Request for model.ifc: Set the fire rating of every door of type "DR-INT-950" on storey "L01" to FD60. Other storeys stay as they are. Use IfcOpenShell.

First a look at what the model holds.

```python
import ifcopenshell
import ifcopenshell.util.element

model = ifcopenshell.open("model.ifc")
print(model.schema)
storey = next(s for s in model.by_type("IfcBuildingStorey") if s.Name == "L01")
doors = [e for e in ifcopenshell.util.element.get_decomposition(storey) if e.is_a("IfcDoor")]
seen = {}
for e in doors:
    element_type = ifcopenshell.util.element.get_type(e)
    key = (element_type.Name if element_type != e and element_type else None, ifcopenshell.util.element.get_pset(e, "Pset_DoorCommon", "FireRating"))
    seen[key] = seen.get(key, 0) + 1
for (name, value), count in sorted(seen.items(), key=str):
    print(count, "x", name, "|", value)
```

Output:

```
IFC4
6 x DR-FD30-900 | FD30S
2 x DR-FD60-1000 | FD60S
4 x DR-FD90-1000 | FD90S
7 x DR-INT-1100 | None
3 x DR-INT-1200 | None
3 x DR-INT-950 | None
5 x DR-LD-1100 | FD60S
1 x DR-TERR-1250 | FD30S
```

```python
import ifcopenshell
import ifcopenshell.api.pset
import ifcopenshell.util.element

model = ifcopenshell.open("model.ifc")

storey = next(s for s in model.by_type("IfcBuildingStorey") if s.Name == "L01")
doors = [e for e in ifcopenshell.util.element.get_decomposition(storey) if e.is_a("IfcDoor")]

count = 0
for e in doors:
    element_type = ifcopenshell.util.element.get_type(e)
    if element_type in (None, e) or element_type.Name != "DR-INT-950":
        continue
    found = ifcopenshell.util.element.get_pset(e, "Pset_DoorCommon", should_inherit=False)
    if found:
        pset = model.by_id(found["id"])
        if len(ifcopenshell.util.element.get_elements_by_pset(pset)) > 1:
            pset = ifcopenshell.api.pset.unshare_pset(model, products=[e], pset=pset)[0]
    else:
        pset = ifcopenshell.api.pset.add_pset(model, product=e, name="Pset_DoorCommon")
    ifcopenshell.api.pset.edit_pset(model, pset=pset, properties={"FireRating": "FD60"})
    count += 1

print(count, "doors updated")

model.write("model_rev.ifc")
```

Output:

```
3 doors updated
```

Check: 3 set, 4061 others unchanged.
